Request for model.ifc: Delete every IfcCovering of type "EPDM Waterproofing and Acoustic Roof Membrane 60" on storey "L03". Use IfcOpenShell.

First a look at what the model holds.

```python
import ifcopenshell
import ifcopenshell.util.element

model = ifcopenshell.open("model.ifc")
print(model.schema)
storey = next(s for s in model.by_type("IfcBuildingStorey") if s.Name == "L03")
coverings = [e for e in ifcopenshell.util.element.get_decomposition(storey) if e.is_a("IfcCovering")]
seen = {}
for e in coverings:
    element_type = ifcopenshell.util.element.get_type(e)
    name = element_type.Name if element_type not in (None, e) else None
    seen[name] = seen.get(name, 0) + 1
for name, count in sorted(seen.items(), key=str):
    print(count, "x", name)
```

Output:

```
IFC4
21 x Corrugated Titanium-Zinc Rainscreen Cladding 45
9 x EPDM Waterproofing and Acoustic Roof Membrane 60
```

```python
import ifcopenshell
import ifcopenshell.api.root
import ifcopenshell.util.element

model = ifcopenshell.open("model.ifc")

storey = next(s for s in model.by_type("IfcBuildingStorey") if s.Name == "L03")
coverings = [e for e in ifcopenshell.util.element.get_decomposition(storey) if e.is_a("IfcCovering")]
targets = [e for e in coverings if (t := ifcopenshell.util.element.get_type(e)) not in (None, e) and t.Name == "EPDM Waterproofing and Acoustic Roof Membrane 60"]

for e in targets:
    ifcopenshell.api.root.remove_product(model, product=e)
print(len(targets), "removed")

model.write("model_updated.ifc")
```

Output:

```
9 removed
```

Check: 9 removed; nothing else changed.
